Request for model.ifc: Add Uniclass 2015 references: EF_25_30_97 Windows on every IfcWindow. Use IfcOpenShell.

First a look at what the model holds.

```python
import ifcopenshell

model = ifcopenshell.open("model.ifc")
print(model.schema)
print("classifications:", [c.Name for c in model.by_type("IfcClassification")])
for ifc_class in ("IfcDoor", "IfcRoof", "IfcStair", "IfcWall", "IfcWindow"):
    print(ifc_class, len(model.by_type(ifc_class)))
```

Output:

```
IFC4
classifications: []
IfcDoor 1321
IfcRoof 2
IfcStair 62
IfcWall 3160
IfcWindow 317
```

```python
import ifcopenshell
import ifcopenshell.api.classification

model = ifcopenshell.open("model.ifc")

system = ifcopenshell.api.classification.add_classification(model, classification="Uniclass 2015")

codes = {
    "IfcWindow": ("EF_25_30_97", "Windows"),
}
for ifc_class, (code, name) in codes.items():
    products = model.by_type(ifc_class)
    ifcopenshell.api.classification.add_reference(
        model, products=products, classification=system, identification=code, name=name
    )
    print(code, len(products))

model.write("model_updated.ifc")
```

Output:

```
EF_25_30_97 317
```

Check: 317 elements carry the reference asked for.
